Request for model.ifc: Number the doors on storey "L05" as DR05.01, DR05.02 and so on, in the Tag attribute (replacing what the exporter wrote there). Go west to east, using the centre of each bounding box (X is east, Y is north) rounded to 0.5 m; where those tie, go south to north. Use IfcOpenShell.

First a look at what the model holds.

```python
import ifcopenshell
import ifcopenshell.util.element
import ifcopenshell.util.placement

model = ifcopenshell.open("model.ifc")
print(model.schema)
storey = next(s for s in model.by_type("IfcBuildingStorey") if s.Name == "L05")
doors = [e for e in ifcopenshell.util.element.get_decomposition(storey) if e.is_a("IfcDoor")]
for e in sorted(doors, key=lambda e: e.id()):
    origin = ifcopenshell.util.placement.get_local_placement(e.ObjectPlacement)[:3, 3]
    print(e.id(), e.Tag, e.Name, origin.round(2) + 0.0, sep=" | ")
```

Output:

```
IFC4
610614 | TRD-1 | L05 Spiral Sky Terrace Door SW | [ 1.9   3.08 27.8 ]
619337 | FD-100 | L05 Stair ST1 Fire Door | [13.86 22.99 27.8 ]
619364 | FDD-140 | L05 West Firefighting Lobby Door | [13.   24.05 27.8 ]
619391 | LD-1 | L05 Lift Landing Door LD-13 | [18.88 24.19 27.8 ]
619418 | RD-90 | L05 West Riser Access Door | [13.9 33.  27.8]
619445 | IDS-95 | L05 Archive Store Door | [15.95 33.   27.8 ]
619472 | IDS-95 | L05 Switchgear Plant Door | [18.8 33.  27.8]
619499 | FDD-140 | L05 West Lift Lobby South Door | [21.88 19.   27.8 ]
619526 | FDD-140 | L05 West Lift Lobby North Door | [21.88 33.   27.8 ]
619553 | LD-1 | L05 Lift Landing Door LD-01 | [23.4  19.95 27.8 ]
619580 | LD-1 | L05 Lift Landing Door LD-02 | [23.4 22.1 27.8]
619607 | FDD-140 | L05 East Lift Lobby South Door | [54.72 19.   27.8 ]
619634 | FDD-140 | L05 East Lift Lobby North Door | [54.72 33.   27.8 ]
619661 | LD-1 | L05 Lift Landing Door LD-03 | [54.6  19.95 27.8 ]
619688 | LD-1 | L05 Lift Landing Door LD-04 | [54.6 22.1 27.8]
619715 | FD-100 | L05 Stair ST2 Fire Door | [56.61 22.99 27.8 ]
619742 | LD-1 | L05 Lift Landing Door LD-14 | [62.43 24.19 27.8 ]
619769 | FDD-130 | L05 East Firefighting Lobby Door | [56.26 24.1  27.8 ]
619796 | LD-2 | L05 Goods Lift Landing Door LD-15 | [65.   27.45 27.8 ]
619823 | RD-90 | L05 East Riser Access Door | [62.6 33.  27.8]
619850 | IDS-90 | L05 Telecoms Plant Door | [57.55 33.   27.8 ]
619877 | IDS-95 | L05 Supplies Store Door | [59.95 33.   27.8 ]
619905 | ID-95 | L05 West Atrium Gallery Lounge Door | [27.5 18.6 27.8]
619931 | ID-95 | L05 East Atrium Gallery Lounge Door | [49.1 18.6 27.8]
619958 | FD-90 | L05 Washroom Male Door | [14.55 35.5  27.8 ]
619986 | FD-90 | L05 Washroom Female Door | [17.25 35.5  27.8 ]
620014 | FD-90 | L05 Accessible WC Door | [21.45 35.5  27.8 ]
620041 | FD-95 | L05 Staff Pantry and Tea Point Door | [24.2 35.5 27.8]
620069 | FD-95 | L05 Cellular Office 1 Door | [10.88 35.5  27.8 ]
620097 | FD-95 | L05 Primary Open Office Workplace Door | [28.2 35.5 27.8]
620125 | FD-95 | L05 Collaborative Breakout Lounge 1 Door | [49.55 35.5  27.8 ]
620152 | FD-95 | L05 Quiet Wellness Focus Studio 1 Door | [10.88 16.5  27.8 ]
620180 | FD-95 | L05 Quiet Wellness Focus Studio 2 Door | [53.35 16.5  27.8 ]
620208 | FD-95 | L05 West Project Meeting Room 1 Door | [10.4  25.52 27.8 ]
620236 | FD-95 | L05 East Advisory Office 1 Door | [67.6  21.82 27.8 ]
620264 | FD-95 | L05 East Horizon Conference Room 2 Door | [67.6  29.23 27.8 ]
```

```python
import ifcopenshell
import ifcopenshell.geom
import ifcopenshell.util.element
import ifcopenshell.util.shape

model = ifcopenshell.open("model.ifc")
settings = ifcopenshell.geom.settings()
settings.set("use-world-coords", True)


def centre(element):
    shape = ifcopenshell.geom.create_shape(settings, element)
    return ifcopenshell.util.shape.get_bbox_centroid(shape.geometry)


storey = next(s for s in model.by_type("IfcBuildingStorey") if s.Name == "L05")
doors = [e for e in ifcopenshell.util.element.get_decomposition(storey) if e.is_a("IfcDoor")]

# Insertion points can sit at a corner or the storey origin, so sort by the geometry (in metres).
centres = {e: centre(e) for e in doors}
doors.sort(key=lambda e: (round(centres[e][0] / 0.5), centres[e][1]))

for i, e in enumerate(doors, start=1):
    number = f"DR05.{i:02d}"
    e.Tag = number
    print(e.id(), number)

model.write("model_updated.ifc")
```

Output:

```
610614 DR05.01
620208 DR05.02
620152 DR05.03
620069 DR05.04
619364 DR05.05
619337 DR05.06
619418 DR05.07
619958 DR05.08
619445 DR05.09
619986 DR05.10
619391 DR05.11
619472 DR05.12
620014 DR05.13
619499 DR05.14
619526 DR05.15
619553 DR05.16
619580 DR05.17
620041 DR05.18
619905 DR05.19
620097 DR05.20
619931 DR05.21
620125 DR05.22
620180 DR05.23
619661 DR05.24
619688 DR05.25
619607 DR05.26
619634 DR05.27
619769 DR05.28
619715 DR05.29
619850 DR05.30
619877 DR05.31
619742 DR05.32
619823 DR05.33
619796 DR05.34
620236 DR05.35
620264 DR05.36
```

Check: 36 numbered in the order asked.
